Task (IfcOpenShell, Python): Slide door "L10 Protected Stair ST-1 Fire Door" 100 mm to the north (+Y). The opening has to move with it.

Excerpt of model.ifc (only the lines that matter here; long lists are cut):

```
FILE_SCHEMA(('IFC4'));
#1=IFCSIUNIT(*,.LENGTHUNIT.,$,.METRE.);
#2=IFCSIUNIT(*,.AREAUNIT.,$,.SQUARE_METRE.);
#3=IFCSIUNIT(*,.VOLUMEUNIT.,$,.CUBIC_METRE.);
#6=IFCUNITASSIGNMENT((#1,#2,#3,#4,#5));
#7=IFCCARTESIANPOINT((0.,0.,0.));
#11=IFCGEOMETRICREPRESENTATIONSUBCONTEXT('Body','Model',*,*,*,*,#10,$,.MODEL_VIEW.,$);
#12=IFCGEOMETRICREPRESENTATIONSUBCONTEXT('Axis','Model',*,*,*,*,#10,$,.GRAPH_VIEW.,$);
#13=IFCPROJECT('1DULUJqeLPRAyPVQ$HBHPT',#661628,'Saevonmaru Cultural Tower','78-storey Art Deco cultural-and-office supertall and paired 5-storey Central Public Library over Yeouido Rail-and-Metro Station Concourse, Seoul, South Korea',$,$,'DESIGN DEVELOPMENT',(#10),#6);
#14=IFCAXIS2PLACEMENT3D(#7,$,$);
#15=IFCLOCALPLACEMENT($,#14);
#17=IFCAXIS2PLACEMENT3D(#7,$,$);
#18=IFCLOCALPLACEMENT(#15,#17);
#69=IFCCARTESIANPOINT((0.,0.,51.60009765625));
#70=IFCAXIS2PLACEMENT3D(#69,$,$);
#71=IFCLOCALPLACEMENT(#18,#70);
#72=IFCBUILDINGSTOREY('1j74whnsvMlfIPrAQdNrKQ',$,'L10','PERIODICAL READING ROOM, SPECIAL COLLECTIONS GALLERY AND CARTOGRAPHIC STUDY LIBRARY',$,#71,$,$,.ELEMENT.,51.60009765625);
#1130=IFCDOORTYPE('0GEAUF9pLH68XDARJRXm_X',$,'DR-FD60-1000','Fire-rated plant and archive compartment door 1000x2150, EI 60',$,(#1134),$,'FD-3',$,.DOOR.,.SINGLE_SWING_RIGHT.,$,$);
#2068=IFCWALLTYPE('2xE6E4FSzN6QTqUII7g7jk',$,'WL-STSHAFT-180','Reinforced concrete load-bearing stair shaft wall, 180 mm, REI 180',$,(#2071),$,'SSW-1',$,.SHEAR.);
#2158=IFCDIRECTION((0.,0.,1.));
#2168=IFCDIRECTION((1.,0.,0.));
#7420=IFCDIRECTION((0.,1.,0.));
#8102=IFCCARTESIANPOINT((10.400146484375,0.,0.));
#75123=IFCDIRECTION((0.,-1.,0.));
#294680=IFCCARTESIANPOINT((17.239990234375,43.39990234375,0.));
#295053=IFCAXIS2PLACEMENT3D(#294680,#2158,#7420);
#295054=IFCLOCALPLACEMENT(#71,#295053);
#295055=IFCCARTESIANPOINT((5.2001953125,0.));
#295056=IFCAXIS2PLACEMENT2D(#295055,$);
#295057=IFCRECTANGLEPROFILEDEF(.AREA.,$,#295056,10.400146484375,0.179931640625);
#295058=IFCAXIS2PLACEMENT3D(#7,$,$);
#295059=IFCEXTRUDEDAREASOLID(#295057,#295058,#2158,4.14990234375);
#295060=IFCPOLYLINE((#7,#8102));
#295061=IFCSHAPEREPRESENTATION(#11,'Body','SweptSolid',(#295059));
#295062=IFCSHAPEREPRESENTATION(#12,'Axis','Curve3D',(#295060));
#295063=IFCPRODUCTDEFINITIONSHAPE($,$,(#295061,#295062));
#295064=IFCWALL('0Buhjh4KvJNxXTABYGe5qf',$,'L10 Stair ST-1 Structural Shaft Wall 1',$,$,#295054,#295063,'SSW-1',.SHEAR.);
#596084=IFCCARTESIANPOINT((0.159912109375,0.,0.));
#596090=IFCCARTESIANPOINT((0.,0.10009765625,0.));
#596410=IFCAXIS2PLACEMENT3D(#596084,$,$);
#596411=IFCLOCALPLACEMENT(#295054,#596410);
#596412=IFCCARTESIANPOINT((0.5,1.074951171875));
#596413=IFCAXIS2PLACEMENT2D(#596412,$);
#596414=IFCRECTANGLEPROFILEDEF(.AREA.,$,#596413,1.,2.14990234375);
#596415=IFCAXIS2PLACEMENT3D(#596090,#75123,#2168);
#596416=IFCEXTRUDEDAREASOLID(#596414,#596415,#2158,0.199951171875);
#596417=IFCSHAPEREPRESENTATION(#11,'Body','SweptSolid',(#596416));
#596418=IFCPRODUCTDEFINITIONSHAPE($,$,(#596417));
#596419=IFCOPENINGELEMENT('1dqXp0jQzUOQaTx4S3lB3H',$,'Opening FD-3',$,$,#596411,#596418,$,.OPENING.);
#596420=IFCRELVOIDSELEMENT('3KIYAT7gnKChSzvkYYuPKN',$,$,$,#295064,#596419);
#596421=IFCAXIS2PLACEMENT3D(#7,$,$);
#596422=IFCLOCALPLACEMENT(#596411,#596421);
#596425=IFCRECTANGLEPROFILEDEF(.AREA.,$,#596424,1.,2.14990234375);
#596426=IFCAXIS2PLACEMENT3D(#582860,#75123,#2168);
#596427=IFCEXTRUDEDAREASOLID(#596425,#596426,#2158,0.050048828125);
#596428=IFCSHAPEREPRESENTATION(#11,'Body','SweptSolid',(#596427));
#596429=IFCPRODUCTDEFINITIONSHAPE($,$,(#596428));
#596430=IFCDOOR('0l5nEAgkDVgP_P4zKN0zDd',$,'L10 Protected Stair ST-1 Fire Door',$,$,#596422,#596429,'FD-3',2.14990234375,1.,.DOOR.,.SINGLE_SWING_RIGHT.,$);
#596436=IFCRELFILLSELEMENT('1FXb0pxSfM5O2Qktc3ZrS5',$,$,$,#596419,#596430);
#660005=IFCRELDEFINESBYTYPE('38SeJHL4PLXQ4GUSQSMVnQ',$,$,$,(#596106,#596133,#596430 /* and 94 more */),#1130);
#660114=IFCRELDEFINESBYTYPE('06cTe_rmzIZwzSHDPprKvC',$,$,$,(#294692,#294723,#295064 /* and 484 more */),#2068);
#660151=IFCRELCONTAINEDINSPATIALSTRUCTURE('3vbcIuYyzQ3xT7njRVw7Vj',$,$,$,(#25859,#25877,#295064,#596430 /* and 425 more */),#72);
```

```python
import ifcopenshell
import ifcopenshell.api.geometry
import ifcopenshell.util.placement

model = ifcopenshell.open("model.ifc")

door = model.by_guid("0l5nEAgkDVgP_P4zKN0zDd")
opening = door.FillsVoids[0].RelatingOpeningElement
wall = opening.VoidsElements[0].RelatingBuildingElement

wall_matrix = ifcopenshell.util.placement.get_local_placement(wall.ObjectPlacement)
shift = wall_matrix[:3, 0] * 0.1
before = ifcopenshell.util.placement.get_local_placement(door.ObjectPlacement)[:3, 3].copy()

# The door is placed relative to its opening, so it follows when the opening moves.
matrix = ifcopenshell.util.placement.get_local_placement(opening.ObjectPlacement)
matrix[:3, 3] += shift
ifcopenshell.api.geometry.edit_object_placement(
    model, product=opening, matrix=matrix, is_si=False, should_transform_children=True
)

after = ifcopenshell.util.placement.get_local_placement(door.ObjectPlacement)[:3, 3]
print("door moved by", (after - before).round(3) + 0.0)

model.write("model-out.ifc")
```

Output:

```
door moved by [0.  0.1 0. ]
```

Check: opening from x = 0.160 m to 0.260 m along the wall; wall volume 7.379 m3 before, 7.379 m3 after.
